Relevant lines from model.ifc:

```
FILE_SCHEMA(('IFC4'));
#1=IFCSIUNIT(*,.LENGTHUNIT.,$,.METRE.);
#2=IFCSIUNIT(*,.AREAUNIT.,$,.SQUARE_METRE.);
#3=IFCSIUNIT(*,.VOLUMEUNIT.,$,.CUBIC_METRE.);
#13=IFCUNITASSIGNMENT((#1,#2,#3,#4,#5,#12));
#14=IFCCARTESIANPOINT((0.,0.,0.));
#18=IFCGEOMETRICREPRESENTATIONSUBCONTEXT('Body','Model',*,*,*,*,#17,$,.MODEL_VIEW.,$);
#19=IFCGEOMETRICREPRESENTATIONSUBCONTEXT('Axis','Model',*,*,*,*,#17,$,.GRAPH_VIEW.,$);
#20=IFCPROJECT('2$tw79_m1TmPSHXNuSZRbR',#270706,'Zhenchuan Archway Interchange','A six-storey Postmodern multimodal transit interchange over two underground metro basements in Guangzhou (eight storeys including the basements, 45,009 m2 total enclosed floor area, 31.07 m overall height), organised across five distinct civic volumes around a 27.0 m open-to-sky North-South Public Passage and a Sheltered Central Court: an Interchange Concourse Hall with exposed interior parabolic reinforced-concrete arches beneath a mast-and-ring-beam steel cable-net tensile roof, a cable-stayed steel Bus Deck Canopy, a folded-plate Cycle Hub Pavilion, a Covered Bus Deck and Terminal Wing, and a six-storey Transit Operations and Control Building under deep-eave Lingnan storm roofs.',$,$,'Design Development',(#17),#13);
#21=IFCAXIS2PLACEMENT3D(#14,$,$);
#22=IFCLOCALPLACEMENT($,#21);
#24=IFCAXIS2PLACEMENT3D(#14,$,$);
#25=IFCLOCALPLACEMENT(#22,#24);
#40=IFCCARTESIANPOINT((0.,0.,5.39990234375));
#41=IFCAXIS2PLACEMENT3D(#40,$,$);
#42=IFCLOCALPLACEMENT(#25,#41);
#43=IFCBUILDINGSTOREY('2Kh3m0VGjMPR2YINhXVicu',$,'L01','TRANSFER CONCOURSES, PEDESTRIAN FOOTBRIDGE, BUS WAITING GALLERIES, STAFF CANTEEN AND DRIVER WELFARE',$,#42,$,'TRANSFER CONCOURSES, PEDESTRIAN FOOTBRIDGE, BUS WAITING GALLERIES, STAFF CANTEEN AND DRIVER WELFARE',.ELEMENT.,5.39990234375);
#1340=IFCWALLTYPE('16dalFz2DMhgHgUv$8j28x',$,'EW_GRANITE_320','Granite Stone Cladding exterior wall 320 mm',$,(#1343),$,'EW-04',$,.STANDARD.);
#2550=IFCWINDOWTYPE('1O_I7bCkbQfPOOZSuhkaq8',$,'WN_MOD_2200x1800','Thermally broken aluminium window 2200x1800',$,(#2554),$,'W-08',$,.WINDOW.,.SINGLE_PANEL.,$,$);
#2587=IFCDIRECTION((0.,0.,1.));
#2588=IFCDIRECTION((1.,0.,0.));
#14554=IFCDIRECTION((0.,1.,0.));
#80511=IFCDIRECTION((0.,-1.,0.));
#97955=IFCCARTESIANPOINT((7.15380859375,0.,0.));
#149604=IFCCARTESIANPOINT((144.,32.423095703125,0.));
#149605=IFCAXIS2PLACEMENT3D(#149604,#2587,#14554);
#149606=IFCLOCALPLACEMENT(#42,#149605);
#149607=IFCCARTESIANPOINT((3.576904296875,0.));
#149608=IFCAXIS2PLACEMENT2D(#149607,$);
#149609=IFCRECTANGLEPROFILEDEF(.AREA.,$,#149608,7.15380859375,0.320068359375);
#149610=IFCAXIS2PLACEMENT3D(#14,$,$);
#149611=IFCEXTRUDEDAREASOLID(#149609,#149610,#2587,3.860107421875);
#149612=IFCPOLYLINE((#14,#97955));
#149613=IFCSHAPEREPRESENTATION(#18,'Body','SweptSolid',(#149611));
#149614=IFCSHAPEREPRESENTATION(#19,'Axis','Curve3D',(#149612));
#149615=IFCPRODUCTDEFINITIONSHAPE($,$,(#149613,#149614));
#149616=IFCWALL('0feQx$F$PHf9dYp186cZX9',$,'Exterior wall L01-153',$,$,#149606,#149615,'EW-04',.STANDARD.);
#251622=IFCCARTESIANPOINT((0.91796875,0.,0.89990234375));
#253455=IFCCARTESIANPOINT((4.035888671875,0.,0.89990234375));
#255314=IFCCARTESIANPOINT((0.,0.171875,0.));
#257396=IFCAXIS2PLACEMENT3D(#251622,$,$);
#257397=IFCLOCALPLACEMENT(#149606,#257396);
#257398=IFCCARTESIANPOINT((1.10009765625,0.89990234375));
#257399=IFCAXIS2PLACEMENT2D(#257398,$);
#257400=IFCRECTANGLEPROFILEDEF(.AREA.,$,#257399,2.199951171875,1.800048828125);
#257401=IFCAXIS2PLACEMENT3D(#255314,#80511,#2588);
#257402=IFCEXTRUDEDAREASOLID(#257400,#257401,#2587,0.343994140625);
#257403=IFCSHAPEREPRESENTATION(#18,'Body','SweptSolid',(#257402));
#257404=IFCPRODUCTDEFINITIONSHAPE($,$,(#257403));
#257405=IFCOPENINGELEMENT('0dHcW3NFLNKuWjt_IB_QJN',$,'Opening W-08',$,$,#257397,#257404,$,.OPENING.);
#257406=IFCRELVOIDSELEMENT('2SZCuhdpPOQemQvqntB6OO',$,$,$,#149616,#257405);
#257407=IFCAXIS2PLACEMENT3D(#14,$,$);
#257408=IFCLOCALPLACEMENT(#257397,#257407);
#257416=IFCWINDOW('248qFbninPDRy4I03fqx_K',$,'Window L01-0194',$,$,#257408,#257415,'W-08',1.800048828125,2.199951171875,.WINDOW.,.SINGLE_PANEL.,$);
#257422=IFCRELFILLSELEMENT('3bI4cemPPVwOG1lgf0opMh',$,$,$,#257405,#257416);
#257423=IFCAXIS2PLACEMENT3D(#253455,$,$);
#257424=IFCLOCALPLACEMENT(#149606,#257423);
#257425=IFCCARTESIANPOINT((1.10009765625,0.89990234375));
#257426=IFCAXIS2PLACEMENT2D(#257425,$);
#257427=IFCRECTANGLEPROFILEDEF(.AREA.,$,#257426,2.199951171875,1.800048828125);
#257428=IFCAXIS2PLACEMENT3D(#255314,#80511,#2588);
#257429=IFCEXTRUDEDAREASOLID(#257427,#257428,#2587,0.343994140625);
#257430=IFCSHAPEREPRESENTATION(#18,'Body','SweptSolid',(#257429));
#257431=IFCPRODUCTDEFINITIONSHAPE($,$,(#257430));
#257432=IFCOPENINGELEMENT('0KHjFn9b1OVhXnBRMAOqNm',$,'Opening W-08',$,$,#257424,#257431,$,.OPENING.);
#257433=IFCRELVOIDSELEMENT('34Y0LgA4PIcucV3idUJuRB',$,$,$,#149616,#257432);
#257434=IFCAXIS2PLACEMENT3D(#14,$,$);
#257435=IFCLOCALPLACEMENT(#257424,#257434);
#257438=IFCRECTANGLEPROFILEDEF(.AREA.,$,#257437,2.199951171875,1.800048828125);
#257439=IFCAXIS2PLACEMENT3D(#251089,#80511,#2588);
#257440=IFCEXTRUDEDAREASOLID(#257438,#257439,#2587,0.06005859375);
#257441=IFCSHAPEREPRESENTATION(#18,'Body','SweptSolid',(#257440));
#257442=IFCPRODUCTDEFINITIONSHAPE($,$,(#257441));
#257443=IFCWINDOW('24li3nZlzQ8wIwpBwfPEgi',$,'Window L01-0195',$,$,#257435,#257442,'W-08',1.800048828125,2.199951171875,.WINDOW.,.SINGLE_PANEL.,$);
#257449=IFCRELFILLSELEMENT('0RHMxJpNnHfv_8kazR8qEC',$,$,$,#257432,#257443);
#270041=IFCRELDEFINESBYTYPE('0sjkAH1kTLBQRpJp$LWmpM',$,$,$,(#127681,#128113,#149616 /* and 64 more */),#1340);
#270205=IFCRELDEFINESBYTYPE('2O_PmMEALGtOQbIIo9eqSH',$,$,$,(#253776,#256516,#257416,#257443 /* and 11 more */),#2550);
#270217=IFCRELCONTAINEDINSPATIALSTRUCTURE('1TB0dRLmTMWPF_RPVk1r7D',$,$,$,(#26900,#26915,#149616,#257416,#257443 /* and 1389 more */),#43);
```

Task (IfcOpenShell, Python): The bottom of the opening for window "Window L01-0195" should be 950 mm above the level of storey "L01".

```python
import numpy as np
import ifcopenshell
import ifcopenshell.api.geometry
import ifcopenshell.geom
import ifcopenshell.util.element
import ifcopenshell.util.placement
import ifcopenshell.util.shape
import ifcopenshell.util.unit

model = ifcopenshell.open("model.ifc")
unit_scale = ifcopenshell.util.unit.calculate_unit_scale(model)

window = model.by_guid("24li3nZlzQ8wIwpBwfPEgi")
opening = window.FillsVoids[0].RelatingOpeningElement
storey = ifcopenshell.util.element.get_container(window, ifc_class="IfcBuildingStorey")
level = ifcopenshell.util.placement.get_local_placement(storey.ObjectPlacement)[2, 3]

# The opening's origin need not be at the sill, so measure its lowest point.
shape = ifcopenshell.geom.create_shape(ifcopenshell.geom.settings(), opening)
bottom = ifcopenshell.util.shape.get_shape_bottom_elevation(shape, shape.geometry) / unit_scale
dz = level + 0.95 / unit_scale - bottom

shift = np.array([0.0, 0.0, dz])
# The window is placed relative to its opening, so it follows when the opening moves.
matrix = ifcopenshell.util.placement.get_local_placement(opening.ObjectPlacement)
matrix[:3, 3] += shift
ifcopenshell.api.geometry.edit_object_placement(
    model, product=opening, matrix=matrix, is_si=False, should_transform_children=True
)

print(f"moved by {dz * unit_scale:+.3f} m")

model.write("model_edited.ifc")
```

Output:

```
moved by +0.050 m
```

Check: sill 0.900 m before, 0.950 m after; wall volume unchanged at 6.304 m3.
